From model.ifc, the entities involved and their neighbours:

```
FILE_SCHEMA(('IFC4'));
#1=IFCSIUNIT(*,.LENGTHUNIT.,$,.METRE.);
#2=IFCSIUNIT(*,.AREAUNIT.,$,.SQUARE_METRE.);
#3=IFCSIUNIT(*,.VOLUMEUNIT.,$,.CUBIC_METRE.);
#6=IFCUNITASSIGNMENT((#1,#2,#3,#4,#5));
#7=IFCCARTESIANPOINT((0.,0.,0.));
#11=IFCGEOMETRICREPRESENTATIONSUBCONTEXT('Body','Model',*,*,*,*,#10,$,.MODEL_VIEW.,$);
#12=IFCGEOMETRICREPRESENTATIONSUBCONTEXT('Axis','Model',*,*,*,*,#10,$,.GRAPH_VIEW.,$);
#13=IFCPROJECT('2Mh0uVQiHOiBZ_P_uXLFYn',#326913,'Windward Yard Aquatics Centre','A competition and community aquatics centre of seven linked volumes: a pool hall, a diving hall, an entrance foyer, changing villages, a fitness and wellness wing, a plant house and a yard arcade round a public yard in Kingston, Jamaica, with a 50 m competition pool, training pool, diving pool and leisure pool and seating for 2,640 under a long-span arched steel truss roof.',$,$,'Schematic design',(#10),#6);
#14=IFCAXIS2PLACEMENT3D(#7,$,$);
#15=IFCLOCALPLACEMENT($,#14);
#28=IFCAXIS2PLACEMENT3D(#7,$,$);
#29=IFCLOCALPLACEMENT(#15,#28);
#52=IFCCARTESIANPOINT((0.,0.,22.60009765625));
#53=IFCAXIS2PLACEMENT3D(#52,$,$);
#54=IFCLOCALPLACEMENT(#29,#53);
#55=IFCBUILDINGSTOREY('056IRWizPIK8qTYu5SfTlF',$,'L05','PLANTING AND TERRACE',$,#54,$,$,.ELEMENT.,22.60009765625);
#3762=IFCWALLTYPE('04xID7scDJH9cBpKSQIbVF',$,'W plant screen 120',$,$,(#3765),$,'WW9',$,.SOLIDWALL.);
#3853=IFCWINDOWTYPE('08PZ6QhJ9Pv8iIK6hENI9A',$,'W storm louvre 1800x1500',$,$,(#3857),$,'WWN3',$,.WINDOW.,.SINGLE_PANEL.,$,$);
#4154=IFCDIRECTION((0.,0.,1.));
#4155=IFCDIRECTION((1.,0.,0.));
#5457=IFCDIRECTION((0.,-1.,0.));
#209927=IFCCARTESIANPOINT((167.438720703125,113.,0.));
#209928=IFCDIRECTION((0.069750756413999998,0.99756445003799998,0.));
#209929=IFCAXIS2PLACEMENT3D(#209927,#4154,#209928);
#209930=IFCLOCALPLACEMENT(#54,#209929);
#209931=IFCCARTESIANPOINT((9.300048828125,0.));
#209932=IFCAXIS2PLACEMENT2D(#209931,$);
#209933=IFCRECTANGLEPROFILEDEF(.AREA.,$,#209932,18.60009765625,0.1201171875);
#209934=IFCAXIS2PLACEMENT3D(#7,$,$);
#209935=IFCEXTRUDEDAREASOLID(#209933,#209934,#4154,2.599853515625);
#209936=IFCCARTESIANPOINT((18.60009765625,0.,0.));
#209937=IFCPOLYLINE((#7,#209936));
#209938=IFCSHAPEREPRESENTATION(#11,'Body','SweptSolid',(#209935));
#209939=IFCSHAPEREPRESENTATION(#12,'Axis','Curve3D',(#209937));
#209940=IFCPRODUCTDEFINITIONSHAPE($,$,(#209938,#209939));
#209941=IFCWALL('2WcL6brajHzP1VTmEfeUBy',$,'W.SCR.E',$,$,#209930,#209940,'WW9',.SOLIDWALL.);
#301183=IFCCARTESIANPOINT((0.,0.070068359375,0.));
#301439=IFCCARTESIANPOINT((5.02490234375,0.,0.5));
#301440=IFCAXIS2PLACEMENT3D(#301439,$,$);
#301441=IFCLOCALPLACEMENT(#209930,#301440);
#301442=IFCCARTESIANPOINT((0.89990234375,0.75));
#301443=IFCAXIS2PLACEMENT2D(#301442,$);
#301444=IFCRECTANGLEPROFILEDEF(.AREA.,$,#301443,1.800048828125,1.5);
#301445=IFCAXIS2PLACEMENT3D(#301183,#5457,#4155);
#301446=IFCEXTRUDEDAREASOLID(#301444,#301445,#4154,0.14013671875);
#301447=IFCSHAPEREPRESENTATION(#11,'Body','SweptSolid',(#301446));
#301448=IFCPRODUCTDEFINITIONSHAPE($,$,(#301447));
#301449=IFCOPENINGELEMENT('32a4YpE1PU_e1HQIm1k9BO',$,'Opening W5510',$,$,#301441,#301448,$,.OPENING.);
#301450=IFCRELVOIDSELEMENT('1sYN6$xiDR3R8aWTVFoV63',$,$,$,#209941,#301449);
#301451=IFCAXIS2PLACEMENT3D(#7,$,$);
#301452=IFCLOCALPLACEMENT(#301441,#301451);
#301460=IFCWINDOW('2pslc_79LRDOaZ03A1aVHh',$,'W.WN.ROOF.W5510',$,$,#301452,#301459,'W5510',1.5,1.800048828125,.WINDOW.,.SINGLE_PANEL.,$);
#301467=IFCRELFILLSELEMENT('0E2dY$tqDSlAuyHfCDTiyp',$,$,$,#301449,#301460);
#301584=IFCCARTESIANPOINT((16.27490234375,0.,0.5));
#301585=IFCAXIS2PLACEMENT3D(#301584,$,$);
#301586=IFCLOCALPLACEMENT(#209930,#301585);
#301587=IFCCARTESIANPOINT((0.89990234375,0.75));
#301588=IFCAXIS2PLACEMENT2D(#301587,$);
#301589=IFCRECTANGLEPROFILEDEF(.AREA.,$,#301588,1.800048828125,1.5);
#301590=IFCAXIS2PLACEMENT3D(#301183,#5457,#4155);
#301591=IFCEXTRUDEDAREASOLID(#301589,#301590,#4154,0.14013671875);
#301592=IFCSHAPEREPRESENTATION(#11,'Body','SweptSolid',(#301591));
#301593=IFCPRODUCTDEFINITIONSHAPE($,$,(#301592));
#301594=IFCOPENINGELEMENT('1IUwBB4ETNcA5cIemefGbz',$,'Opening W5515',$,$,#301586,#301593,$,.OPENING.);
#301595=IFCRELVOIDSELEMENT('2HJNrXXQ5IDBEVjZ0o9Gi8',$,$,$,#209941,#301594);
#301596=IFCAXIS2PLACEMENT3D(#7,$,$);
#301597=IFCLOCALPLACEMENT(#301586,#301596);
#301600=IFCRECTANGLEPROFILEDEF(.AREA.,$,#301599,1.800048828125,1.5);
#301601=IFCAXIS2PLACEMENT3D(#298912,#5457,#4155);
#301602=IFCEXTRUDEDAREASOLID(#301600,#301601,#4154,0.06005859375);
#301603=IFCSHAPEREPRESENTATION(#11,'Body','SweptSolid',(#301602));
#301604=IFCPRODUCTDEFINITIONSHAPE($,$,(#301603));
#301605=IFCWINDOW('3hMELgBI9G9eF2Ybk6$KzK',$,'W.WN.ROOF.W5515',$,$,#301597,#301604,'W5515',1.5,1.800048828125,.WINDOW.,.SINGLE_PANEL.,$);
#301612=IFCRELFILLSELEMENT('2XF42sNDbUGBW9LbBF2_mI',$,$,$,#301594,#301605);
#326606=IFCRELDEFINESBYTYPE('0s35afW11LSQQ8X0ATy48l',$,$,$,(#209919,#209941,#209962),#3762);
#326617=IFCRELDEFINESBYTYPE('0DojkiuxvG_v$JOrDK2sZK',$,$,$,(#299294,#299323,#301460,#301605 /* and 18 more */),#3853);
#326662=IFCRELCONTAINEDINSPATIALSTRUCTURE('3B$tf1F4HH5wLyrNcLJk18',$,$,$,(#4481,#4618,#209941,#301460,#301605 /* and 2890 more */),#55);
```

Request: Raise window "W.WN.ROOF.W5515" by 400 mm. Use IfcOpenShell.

```python
import numpy as np
import ifcopenshell
import ifcopenshell.api.geometry
import ifcopenshell.util.placement
import ifcopenshell.util.unit

model = ifcopenshell.open("model.ifc")
unit_scale = ifcopenshell.util.unit.calculate_unit_scale(model)

window = model.by_guid("3hMELgBI9G9eF2Ybk6$KzK")
opening = window.FillsVoids[0].RelatingOpeningElement
dz = 0.4 / unit_scale

shift = np.array([0.0, 0.0, dz])
# The window is placed relative to its opening, so it follows when the opening moves.
matrix = ifcopenshell.util.placement.get_local_placement(opening.ObjectPlacement)
matrix[:3, 3] += shift
ifcopenshell.api.geometry.edit_object_placement(
    model, product=opening, matrix=matrix, is_si=False, should_transform_children=True
)

print(f"moved by {dz * unit_scale:+.3f} m")

model.write("model_rev.ifc")
```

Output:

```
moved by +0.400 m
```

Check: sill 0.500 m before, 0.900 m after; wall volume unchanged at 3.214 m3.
